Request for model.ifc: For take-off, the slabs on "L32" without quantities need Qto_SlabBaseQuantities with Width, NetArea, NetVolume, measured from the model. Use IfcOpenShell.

First a look at what the model holds.

```python
import ifcopenshell
import ifcopenshell.util.element
import ifcopenshell.util.unit

model = ifcopenshell.open("model.ifc")
print(model.schema)
for unit_type in ("LENGTHUNIT", "AREAUNIT", "VOLUMEUNIT"):
    print(unit_type, ifcopenshell.util.unit.calculate_unit_scale(model, unit_type))
storey = next(s for s in model.by_type("IfcBuildingStorey") if s.Name == "L32")
slabs = [e for e in ifcopenshell.util.element.get_decomposition(storey) if e.is_a("IfcSlab")]
for e in sorted(slabs, key=lambda e: e.id()):
    print(e.id(), e.is_a(), e.Name, list(ifcopenshell.util.element.get_psets(e, qtos_only=True)), sep=" | ")
```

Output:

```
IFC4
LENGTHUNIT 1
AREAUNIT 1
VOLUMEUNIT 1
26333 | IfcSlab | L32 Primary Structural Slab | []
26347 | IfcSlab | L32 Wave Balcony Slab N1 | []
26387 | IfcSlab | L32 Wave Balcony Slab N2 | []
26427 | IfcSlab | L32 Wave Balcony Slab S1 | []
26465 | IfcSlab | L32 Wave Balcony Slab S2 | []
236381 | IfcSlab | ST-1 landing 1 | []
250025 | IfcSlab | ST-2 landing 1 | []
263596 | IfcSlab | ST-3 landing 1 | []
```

```python
import ifcopenshell
import ifcopenshell.api.pset
import ifcopenshell.geom
import ifcopenshell.util.element
import ifcopenshell.util.shape
import ifcopenshell.util.unit

model = ifcopenshell.open("model.ifc")
unit_scale = ifcopenshell.util.unit.calculate_unit_scale(model)
area_scale = ifcopenshell.util.unit.calculate_unit_scale(model, "AREAUNIT")
volume_scale = ifcopenshell.util.unit.calculate_unit_scale(model, "VOLUMEUNIT")
settings = ifcopenshell.geom.settings()

storey = next(s for s in model.by_type("IfcBuildingStorey") if s.Name == "L32")
slabs = [e for e in ifcopenshell.util.element.get_decomposition(storey) if e.is_a("IfcSlab")]

for e in sorted(slabs, key=lambda e: e.id()):
    if ifcopenshell.util.element.get_psets(e, qtos_only=True, should_inherit=False):
        continue
    # Geometry comes back in metres, in the element's own axes.
    shape = ifcopenshell.geom.create_shape(settings, e)
    values = {
        "Width": ifcopenshell.util.shape.get_z(shape.geometry) / unit_scale,
        "NetArea": ifcopenshell.util.shape.get_footprint_area(shape.geometry) / area_scale,
        "NetVolume": ifcopenshell.util.shape.get_volume(shape.geometry) / volume_scale,
    }
    qto = ifcopenshell.api.pset.add_qto(model, product=e, name="Qto_SlabBaseQuantities")
    ifcopenshell.api.pset.edit_qto(model, qto=qto, properties=values)
    print(e.id(), {k: round(v, 3) for k, v in values.items()})

model.write("model_edited.ifc")
```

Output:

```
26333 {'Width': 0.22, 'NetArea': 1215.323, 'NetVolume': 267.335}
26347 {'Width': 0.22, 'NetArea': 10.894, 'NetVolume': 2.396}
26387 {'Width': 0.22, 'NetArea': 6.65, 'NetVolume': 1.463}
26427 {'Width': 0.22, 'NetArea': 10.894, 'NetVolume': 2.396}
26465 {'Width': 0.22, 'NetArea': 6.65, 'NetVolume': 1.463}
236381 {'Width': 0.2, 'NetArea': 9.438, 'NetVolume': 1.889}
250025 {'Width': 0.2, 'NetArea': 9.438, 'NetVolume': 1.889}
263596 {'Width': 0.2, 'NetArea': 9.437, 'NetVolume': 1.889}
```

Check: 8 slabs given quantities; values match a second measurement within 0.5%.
